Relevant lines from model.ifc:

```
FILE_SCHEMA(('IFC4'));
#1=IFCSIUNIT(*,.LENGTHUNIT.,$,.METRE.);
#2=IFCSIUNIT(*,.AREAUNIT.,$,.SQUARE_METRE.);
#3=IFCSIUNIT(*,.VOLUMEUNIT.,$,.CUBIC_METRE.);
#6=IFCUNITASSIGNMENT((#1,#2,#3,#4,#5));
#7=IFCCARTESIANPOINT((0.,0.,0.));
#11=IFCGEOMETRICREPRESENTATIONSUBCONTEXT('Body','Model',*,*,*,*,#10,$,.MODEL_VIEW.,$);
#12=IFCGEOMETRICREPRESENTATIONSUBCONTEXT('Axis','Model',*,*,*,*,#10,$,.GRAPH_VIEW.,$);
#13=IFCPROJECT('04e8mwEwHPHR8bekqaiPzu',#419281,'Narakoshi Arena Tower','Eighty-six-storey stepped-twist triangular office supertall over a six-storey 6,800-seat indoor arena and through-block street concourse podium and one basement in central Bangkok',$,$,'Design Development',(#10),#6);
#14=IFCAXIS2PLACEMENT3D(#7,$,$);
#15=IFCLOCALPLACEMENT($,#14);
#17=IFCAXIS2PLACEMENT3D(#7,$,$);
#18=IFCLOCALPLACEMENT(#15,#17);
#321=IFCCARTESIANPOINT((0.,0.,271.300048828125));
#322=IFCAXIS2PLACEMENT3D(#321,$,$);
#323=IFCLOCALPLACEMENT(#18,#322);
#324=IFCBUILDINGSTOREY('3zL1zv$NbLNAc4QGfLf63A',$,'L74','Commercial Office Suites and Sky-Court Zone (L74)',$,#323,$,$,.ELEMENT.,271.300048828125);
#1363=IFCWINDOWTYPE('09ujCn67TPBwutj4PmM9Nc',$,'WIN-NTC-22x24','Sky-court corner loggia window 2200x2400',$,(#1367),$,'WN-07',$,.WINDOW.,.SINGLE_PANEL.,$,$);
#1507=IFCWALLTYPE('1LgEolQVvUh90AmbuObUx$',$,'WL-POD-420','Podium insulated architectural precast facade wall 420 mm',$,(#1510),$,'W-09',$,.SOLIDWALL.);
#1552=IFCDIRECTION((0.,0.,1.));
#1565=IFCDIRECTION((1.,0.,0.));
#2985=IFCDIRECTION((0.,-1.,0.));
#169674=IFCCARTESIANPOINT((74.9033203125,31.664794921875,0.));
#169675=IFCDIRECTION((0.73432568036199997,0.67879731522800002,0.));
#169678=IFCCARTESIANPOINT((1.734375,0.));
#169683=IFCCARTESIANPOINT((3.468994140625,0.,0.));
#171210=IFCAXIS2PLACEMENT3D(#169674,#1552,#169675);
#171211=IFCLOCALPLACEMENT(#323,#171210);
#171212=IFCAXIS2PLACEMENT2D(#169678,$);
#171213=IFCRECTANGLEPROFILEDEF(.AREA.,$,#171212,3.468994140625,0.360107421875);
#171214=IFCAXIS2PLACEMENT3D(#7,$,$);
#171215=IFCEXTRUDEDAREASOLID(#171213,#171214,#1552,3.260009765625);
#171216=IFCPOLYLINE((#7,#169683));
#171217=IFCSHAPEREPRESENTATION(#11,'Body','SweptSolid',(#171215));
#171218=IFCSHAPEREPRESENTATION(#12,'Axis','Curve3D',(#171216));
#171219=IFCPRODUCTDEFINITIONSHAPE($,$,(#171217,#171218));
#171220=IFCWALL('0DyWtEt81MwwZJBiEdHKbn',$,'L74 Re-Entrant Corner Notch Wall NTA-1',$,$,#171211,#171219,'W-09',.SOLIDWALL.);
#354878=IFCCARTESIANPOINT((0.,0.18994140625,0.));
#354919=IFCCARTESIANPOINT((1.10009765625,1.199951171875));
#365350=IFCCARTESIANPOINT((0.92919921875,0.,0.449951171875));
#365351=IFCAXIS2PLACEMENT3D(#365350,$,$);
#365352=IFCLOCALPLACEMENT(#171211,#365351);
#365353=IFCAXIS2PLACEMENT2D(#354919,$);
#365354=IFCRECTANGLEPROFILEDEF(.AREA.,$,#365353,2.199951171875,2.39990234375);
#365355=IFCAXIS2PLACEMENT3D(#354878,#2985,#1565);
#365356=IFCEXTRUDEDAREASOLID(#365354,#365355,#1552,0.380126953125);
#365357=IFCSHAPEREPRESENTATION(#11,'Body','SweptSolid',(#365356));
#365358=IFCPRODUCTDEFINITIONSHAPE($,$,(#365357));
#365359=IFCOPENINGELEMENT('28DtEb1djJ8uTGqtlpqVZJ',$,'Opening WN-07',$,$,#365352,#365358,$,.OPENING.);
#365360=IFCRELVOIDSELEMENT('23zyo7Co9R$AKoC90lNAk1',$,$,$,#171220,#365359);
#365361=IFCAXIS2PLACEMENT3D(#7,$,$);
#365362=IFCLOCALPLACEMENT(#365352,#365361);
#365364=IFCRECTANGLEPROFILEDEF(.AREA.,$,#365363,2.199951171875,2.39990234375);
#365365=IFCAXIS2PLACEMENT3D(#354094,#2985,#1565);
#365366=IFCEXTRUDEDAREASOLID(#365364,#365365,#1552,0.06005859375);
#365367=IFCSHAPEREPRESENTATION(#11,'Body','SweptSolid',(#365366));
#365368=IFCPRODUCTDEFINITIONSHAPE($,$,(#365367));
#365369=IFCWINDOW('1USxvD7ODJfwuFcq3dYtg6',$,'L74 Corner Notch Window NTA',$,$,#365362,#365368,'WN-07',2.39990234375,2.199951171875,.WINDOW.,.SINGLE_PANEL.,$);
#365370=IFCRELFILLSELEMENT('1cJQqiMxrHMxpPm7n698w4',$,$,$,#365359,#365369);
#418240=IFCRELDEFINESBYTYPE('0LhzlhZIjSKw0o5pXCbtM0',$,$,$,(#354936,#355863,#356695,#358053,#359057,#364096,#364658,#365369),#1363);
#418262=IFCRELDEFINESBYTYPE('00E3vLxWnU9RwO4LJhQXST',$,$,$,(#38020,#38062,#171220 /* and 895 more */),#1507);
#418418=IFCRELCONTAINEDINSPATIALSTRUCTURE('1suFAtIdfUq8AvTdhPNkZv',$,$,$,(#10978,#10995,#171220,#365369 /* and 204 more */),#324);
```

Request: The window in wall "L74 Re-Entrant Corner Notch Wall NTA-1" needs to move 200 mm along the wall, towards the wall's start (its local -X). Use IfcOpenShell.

```python
import ifcopenshell
import ifcopenshell.api.geometry
import ifcopenshell.util.placement
import ifcopenshell.util.unit

model = ifcopenshell.open("model.ifc")
unit_scale = ifcopenshell.util.unit.calculate_unit_scale(model)

window = model.by_id(365369)
opening = window.FillsVoids[0].RelatingOpeningElement
wall = opening.VoidsElements[0].RelatingBuildingElement

wall_matrix = ifcopenshell.util.placement.get_local_placement(wall.ObjectPlacement)
shift = wall_matrix[:3, 0] * -0.2 / unit_scale
before = ifcopenshell.util.placement.get_local_placement(window.ObjectPlacement)[:3, 3].copy()

# The window is placed relative to its opening, so it follows when the opening moves.
matrix = ifcopenshell.util.placement.get_local_placement(opening.ObjectPlacement)
matrix[:3, 3] += shift
ifcopenshell.api.geometry.edit_object_placement(
    model, product=opening, matrix=matrix, is_si=False, should_transform_children=True
)

after = ifcopenshell.util.placement.get_local_placement(window.ObjectPlacement)[:3, 3]
print("window moved by", (after - before).round(3) + 0.0)

model.write("model_v2.ifc")
```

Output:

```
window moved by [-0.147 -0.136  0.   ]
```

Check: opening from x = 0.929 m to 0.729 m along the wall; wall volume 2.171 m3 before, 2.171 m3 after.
